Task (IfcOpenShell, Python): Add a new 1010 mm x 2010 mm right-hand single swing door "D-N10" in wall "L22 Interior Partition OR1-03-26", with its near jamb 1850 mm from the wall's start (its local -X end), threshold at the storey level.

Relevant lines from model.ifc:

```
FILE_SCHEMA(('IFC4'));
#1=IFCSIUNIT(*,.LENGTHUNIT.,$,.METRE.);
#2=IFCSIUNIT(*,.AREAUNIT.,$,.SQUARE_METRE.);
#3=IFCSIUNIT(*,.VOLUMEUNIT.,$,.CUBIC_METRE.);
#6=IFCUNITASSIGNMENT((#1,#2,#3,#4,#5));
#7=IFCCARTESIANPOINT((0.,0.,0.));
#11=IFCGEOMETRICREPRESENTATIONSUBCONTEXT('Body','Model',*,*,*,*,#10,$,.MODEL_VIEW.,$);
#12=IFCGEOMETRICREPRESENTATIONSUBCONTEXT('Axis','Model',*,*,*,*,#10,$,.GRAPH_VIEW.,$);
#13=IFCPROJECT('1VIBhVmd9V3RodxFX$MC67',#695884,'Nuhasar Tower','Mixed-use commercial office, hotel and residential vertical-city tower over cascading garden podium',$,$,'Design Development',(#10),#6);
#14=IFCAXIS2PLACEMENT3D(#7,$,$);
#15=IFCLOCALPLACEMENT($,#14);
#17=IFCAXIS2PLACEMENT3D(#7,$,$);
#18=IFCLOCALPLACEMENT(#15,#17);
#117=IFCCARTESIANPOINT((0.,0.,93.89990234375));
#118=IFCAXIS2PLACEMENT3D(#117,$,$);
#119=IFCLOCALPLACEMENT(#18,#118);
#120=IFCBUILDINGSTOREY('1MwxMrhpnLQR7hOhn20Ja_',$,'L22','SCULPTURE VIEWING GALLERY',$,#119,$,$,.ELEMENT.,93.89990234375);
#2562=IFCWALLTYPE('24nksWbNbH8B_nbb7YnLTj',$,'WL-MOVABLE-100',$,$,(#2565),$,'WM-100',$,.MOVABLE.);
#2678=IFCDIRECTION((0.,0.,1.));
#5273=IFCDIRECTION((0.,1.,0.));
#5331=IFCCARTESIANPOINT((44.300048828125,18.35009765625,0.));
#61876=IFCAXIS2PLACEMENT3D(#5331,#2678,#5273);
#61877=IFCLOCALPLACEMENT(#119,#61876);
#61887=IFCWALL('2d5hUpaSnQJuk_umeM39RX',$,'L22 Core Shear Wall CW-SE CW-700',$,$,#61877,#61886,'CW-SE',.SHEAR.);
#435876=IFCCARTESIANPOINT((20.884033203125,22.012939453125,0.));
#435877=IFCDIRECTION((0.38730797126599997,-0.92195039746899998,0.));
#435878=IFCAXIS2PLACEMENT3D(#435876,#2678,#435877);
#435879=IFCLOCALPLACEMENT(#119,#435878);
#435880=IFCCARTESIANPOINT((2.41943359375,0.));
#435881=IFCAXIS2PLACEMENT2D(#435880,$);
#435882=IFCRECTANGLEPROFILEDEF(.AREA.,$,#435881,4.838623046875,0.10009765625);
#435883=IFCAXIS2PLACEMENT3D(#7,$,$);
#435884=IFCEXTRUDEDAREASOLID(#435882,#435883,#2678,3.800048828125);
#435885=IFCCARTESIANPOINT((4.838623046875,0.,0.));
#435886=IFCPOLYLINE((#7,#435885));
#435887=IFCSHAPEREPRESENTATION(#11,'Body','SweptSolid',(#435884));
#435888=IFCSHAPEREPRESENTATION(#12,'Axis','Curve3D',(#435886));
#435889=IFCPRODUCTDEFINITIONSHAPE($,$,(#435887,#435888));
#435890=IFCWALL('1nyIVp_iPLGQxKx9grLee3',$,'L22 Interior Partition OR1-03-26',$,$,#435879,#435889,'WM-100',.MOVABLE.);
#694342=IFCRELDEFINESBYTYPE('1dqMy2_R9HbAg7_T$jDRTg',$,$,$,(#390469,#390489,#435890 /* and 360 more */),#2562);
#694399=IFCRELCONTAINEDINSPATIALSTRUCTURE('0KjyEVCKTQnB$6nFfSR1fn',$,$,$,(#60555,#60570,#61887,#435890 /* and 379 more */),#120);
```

```python
import numpy as np
import ifcopenshell
import ifcopenshell.api.feature
import ifcopenshell.api.geometry
import ifcopenshell.api.root
import ifcopenshell.api.spatial
import ifcopenshell.geom
import ifcopenshell.util.element
import ifcopenshell.util.placement
import ifcopenshell.util.representation
import ifcopenshell.util.shape
import ifcopenshell.util.unit

model = ifcopenshell.open("model.ifc")
unit_scale = ifcopenshell.util.unit.calculate_unit_scale(model)
settings = ifcopenshell.geom.settings()


def volume(element):
    """Net volume in cubic metres, openings subtracted."""
    shape = ifcopenshell.geom.create_shape(settings, element)
    return ifcopenshell.util.shape.get_volume(shape.geometry)


wall = model.by_guid("1nyIVp_iPLGQxKx9grLee3")
storey = ifcopenshell.util.element.get_container(wall, ifc_class="IfcBuildingStorey")
context = ifcopenshell.util.representation.get_context(model, "Model", "Body", "MODEL_VIEW")
before = volume(wall)

width, height, from_end, sill = 1.01, 2.01, 1.85, 0.0  # metres

# The wall runs along its own X axis, and the end named is its -X end.
wall_shape = ifcopenshell.geom.create_shape(settings, wall)
x, y, z = ifcopenshell.util.shape.get_vertices(wall_shape.geometry).T
start = x.min() + from_end
face, thickness = float(y.min()), float(y.max() - y.min())
wall_matrix = ifcopenshell.util.placement.get_local_placement(wall.ObjectPlacement)
level = ifcopenshell.util.placement.get_local_placement(storey.ObjectPlacement)[2, 3]


def in_wall(x, y):
    """Placement at x, y metres in the wall's axes, at sill height."""
    matrix = wall_matrix.copy()
    matrix[:, 3] = wall_matrix @ np.array([x / unit_scale, y / unit_scale, 0.0, 1.0])
    matrix[2, 3] = level + sill / unit_scale
    return matrix


# Opening: a box that overshoots both wall faces by 50 mm.
opening = ifcopenshell.api.root.create_entity(model, ifc_class="IfcOpeningElement", predefined_type="OPENING")
box = ifcopenshell.api.geometry.add_wall_representation(
    model, context=context, length=width, height=height, thickness=thickness + 0.1
)
ifcopenshell.api.geometry.assign_representation(model, product=opening, representation=box)
ifcopenshell.api.geometry.edit_object_placement(model, product=opening, matrix=in_wall(start, face - 0.05), is_si=False)
ifcopenshell.api.feature.add_feature(model, feature=opening, element=wall)

door = ifcopenshell.api.root.create_entity(model, ifc_class="IfcDoor", name="D-N10", predefined_type="DOOR")
door.OverallWidth, door.OverallHeight = width / unit_scale, height / unit_scale
door.OperationType = "SINGLE_SWING_RIGHT"
body = ifcopenshell.api.geometry.add_door_representation(
    model,
    context=context,
    overall_width=door.OverallWidth,
    overall_height=door.OverallHeight,
    operation_type="SINGLE_SWING_RIGHT",
    lining_properties={"LiningDepth": thickness / unit_scale, "ThresholdDepth": thickness / unit_scale},
)
ifcopenshell.api.geometry.assign_representation(model, product=door, representation=body)
ifcopenshell.api.spatial.assign_container(model, products=[door], relating_structure=storey)
ifcopenshell.api.feature.add_filling(model, opening=opening, element=door)

# The lining spans the wall, so the door starts at the wall face.
ifcopenshell.api.geometry.edit_object_placement(model, product=door, matrix=in_wall(start, face), is_si=False)

after = volume(wall)

print(f"wall volume {before:.3f} -> {after:.3f} m3")

model.write("model_v2.ifc")
```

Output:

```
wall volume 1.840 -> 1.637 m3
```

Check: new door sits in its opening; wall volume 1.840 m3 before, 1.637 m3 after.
